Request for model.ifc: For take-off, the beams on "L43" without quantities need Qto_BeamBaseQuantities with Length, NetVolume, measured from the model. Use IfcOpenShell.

First a look at what the model holds.

```python
import ifcopenshell
import ifcopenshell.util.element
import ifcopenshell.util.unit

model = ifcopenshell.open("model.ifc")
print(model.schema)
for unit_type in ("LENGTHUNIT", "AREAUNIT", "VOLUMEUNIT"):
    print(unit_type, ifcopenshell.util.unit.calculate_unit_scale(model, unit_type))
storey = next(s for s in model.by_type("IfcBuildingStorey") if s.Name == "L43")
beams = [e for e in ifcopenshell.util.element.get_decomposition(storey) if e.is_a("IfcBeam")]
for e in sorted(beams, key=lambda e: e.id()):
    print(e.id(), e.is_a(), e.Name, list(ifcopenshell.util.element.get_psets(e, qtos_only=True)), sep=" | ")
```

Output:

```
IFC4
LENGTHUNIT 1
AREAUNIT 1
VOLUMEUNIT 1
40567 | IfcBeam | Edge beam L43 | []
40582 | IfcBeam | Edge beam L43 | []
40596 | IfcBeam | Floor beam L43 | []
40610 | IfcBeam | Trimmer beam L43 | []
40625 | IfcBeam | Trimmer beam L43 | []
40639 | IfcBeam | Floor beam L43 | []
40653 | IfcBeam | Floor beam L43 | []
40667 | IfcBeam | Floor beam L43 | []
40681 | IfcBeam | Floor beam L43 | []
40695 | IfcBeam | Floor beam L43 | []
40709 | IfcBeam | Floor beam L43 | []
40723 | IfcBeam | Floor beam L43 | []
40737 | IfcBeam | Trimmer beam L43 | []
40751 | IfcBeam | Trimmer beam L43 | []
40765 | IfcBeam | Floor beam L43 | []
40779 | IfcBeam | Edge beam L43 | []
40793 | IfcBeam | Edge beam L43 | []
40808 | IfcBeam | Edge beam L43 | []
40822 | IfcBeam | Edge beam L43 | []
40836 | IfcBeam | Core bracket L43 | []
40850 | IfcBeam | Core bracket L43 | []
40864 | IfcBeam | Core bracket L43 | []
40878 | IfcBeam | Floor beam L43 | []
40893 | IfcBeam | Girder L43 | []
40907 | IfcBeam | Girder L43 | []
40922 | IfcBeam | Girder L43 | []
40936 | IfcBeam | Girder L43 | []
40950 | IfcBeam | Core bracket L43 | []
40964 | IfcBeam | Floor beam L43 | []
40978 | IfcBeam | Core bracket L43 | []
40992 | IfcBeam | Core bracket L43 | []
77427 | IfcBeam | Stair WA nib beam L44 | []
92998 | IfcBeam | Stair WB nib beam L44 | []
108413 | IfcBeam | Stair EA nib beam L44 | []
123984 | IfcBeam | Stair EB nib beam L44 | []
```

```python
import ifcopenshell
import ifcopenshell.api.pset
import ifcopenshell.geom
import ifcopenshell.util.element
import ifcopenshell.util.shape
import ifcopenshell.util.unit

model = ifcopenshell.open("model.ifc")
unit_scale = ifcopenshell.util.unit.calculate_unit_scale(model)
volume_scale = ifcopenshell.util.unit.calculate_unit_scale(model, "VOLUMEUNIT")
settings = ifcopenshell.geom.settings()

storey = next(s for s in model.by_type("IfcBuildingStorey") if s.Name == "L43")
beams = [e for e in ifcopenshell.util.element.get_decomposition(storey) if e.is_a("IfcBeam")]

for e in sorted(beams, key=lambda e: e.id()):
    if ifcopenshell.util.element.get_psets(e, qtos_only=True, should_inherit=False):
        continue
    # Geometry comes back in metres, in the element's own axes.
    shape = ifcopenshell.geom.create_shape(settings, e)
    values = {
        "Length": ifcopenshell.util.shape.get_max_xyz(shape.geometry) / unit_scale,
        "NetVolume": ifcopenshell.util.shape.get_volume(shape.geometry) / volume_scale,
    }
    qto = ifcopenshell.api.pset.add_qto(model, product=e, name="Qto_BeamBaseQuantities")
    ifcopenshell.api.pset.edit_qto(model, qto=qto, properties=values)
    print(e.id(), {k: round(v, 3) for k, v in values.items()})

model.write("model_v2.ifc")
```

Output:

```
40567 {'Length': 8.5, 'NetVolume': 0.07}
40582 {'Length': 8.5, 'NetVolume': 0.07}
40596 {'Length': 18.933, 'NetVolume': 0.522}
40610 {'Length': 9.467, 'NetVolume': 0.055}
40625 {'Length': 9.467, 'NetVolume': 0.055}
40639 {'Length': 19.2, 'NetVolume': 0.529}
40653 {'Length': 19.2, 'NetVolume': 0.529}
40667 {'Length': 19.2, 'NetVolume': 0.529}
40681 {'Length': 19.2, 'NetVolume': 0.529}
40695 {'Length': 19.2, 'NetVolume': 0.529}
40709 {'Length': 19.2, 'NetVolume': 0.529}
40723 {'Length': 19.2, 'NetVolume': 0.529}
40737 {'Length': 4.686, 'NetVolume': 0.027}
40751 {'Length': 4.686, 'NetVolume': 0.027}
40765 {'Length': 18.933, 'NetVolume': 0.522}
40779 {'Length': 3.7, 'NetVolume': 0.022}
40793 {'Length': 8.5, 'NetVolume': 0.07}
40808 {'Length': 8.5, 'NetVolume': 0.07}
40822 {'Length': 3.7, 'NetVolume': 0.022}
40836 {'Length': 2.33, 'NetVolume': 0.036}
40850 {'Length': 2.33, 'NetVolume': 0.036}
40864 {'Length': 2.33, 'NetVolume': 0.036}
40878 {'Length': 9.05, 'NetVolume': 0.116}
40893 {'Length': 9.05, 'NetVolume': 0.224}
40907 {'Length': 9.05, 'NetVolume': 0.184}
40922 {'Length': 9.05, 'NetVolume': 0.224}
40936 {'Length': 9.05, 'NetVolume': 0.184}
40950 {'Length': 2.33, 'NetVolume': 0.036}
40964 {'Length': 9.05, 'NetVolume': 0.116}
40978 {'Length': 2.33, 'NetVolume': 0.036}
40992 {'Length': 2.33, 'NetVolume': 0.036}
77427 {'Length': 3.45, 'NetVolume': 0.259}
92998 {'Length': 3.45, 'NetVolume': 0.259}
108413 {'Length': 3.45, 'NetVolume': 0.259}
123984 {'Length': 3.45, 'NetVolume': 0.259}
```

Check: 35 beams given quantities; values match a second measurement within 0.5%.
